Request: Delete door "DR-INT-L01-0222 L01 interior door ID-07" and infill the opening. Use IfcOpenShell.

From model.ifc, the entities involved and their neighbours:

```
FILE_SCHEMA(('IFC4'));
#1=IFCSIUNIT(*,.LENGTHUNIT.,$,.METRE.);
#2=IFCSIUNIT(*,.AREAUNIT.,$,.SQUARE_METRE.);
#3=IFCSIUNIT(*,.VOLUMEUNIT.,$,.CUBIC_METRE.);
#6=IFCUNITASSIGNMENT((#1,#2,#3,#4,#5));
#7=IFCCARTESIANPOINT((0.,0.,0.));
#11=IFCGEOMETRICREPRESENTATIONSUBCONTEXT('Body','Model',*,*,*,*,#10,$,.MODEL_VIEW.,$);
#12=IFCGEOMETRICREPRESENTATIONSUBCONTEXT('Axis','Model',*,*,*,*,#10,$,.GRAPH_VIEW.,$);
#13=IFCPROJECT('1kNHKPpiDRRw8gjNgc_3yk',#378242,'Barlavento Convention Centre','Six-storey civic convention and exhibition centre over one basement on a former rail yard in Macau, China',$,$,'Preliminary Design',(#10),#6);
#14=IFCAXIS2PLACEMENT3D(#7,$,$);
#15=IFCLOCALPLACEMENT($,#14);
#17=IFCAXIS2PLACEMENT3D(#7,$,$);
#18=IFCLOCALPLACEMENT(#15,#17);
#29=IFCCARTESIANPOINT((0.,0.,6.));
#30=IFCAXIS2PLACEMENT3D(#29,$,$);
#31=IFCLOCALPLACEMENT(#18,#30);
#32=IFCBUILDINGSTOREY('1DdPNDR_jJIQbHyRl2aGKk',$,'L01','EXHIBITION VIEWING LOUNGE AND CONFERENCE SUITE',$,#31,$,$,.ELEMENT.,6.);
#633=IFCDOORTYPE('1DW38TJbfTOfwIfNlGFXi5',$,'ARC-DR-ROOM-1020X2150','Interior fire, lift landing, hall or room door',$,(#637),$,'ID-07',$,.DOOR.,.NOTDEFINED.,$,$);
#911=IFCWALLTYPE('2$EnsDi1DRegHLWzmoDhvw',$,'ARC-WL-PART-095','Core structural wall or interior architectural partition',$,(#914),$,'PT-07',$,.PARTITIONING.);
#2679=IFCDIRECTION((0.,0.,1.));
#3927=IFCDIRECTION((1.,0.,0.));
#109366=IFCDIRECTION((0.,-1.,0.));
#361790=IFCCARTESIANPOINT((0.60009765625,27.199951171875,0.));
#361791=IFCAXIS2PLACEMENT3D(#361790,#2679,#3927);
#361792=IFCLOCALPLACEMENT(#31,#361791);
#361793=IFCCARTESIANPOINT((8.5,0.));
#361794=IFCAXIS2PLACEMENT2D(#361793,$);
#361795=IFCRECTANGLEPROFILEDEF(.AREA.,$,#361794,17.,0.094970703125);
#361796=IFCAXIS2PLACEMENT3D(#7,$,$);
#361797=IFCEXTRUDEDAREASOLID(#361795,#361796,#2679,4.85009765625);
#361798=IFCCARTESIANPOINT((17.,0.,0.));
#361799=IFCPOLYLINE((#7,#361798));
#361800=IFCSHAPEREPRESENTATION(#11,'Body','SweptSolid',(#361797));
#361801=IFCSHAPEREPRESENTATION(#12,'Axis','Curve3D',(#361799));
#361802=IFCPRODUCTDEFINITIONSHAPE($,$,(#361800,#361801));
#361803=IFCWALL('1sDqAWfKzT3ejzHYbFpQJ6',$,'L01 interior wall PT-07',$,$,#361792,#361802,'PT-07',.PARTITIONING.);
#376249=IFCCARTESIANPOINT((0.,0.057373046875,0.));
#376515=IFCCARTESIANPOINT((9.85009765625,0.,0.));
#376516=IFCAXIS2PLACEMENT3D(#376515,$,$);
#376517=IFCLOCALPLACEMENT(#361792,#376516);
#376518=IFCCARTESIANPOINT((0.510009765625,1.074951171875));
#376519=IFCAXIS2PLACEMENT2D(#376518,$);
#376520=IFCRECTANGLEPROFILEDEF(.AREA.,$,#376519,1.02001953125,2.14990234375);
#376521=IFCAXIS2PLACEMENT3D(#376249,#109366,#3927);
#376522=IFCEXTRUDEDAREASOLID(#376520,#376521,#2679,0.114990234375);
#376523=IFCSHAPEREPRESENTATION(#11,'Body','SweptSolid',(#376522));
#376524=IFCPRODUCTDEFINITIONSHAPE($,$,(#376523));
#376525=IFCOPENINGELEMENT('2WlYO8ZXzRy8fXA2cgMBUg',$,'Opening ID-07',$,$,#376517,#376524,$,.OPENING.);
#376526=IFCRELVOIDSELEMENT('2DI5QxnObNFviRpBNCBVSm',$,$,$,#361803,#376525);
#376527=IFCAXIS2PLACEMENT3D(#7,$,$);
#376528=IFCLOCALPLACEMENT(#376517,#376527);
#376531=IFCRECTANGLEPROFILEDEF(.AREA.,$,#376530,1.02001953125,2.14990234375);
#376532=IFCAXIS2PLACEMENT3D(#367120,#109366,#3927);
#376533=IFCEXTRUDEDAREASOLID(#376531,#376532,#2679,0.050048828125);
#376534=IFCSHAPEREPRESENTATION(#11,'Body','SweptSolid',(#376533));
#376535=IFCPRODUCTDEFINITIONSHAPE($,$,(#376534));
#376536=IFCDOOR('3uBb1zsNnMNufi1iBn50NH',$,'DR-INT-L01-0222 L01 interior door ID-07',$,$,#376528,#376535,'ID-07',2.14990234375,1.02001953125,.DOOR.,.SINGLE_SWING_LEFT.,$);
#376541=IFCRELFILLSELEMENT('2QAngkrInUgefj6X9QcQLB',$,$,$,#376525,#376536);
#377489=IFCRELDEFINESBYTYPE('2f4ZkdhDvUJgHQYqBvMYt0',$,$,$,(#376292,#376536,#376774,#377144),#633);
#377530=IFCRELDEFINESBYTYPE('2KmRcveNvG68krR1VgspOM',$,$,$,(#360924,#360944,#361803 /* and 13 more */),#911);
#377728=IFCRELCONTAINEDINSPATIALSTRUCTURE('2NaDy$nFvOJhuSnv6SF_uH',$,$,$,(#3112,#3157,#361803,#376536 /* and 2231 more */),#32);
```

```python
import ifcopenshell
import ifcopenshell.api.feature
import ifcopenshell.api.root
import ifcopenshell.geom
import ifcopenshell.util.shape

model = ifcopenshell.open("model.ifc")
settings = ifcopenshell.geom.settings()


def volume(element):
    """Net volume in cubic metres, openings subtracted."""
    shape = ifcopenshell.geom.create_shape(settings, element)
    return ifcopenshell.util.shape.get_volume(shape.geometry)


door = model.by_guid("3uBb1zsNnMNufi1iBn50NH")
opening = door.FillsVoids[0].RelatingOpeningElement
wall = opening.VoidsElements[0].RelatingBuildingElement
before = volume(wall)

ifcopenshell.api.root.remove_product(model, product=door)
ifcopenshell.api.feature.remove_feature(model, feature=opening)

after = volume(wall)

print(f"wall volume {before:.3f} -> {after:.3f} m3")

model.write("model_rev.ifc")
```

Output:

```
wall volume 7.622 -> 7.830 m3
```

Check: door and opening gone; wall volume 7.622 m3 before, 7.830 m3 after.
